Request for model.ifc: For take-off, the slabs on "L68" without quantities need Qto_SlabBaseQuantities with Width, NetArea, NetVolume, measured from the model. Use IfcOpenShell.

First a look at what the model holds.

```python
import ifcopenshell
import ifcopenshell.util.element
import ifcopenshell.util.unit

model = ifcopenshell.open("model.ifc")
print(model.schema)
for unit_type in ("LENGTHUNIT", "AREAUNIT", "VOLUMEUNIT"):
    print(unit_type, ifcopenshell.util.unit.calculate_unit_scale(model, unit_type))
storey = next(s for s in model.by_type("IfcBuildingStorey") if s.Name == "L68")
slabs = [e for e in ifcopenshell.util.element.get_decomposition(storey) if e.is_a("IfcSlab")]
for e in sorted(slabs, key=lambda e: e.id()):
    print(e.id(), e.is_a(), e.Name, list(ifcopenshell.util.element.get_psets(e, qtos_only=True)), sep=" | ")
```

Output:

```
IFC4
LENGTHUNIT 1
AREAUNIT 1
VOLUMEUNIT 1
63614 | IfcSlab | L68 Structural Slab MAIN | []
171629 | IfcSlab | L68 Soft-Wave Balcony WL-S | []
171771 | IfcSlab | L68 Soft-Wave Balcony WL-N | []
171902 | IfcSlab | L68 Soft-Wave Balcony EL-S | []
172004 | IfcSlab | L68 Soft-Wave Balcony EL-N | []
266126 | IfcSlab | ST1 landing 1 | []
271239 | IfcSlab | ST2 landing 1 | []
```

```python
import ifcopenshell
import ifcopenshell.api.pset
import ifcopenshell.geom
import ifcopenshell.util.element
import ifcopenshell.util.shape
import ifcopenshell.util.unit

model = ifcopenshell.open("model.ifc")
unit_scale = ifcopenshell.util.unit.calculate_unit_scale(model)
area_scale = ifcopenshell.util.unit.calculate_unit_scale(model, "AREAUNIT")
volume_scale = ifcopenshell.util.unit.calculate_unit_scale(model, "VOLUMEUNIT")
settings = ifcopenshell.geom.settings()

storey = next(s for s in model.by_type("IfcBuildingStorey") if s.Name == "L68")
slabs = [e for e in ifcopenshell.util.element.get_decomposition(storey) if e.is_a("IfcSlab")]

for e in sorted(slabs, key=lambda e: e.id()):
    if ifcopenshell.util.element.get_psets(e, qtos_only=True, should_inherit=False):
        continue
    # Geometry comes back in metres, in the element's own axes.
    shape = ifcopenshell.geom.create_shape(settings, e)
    values = {
        "Width": ifcopenshell.util.shape.get_z(shape.geometry) / unit_scale,
        "NetArea": ifcopenshell.util.shape.get_footprint_area(shape.geometry) / area_scale,
        "NetVolume": ifcopenshell.util.shape.get_volume(shape.geometry) / volume_scale,
    }
    qto = ifcopenshell.api.pset.add_qto(model, product=e, name="Qto_SlabBaseQuantities")
    ifcopenshell.api.pset.edit_qto(model, qto=qto, properties=values)
    print(e.id(), {k: round(v, 3) for k, v in values.items()})

model.write("model_rev.ifc")
```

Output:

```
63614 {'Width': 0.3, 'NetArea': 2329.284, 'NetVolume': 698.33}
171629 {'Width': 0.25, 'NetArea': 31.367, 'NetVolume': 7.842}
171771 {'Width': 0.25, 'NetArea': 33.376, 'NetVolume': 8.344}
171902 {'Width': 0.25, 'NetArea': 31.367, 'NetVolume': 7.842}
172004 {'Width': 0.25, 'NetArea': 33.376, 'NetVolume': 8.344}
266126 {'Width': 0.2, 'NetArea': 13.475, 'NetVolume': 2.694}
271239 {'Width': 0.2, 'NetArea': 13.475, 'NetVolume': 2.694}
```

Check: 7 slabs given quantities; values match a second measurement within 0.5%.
